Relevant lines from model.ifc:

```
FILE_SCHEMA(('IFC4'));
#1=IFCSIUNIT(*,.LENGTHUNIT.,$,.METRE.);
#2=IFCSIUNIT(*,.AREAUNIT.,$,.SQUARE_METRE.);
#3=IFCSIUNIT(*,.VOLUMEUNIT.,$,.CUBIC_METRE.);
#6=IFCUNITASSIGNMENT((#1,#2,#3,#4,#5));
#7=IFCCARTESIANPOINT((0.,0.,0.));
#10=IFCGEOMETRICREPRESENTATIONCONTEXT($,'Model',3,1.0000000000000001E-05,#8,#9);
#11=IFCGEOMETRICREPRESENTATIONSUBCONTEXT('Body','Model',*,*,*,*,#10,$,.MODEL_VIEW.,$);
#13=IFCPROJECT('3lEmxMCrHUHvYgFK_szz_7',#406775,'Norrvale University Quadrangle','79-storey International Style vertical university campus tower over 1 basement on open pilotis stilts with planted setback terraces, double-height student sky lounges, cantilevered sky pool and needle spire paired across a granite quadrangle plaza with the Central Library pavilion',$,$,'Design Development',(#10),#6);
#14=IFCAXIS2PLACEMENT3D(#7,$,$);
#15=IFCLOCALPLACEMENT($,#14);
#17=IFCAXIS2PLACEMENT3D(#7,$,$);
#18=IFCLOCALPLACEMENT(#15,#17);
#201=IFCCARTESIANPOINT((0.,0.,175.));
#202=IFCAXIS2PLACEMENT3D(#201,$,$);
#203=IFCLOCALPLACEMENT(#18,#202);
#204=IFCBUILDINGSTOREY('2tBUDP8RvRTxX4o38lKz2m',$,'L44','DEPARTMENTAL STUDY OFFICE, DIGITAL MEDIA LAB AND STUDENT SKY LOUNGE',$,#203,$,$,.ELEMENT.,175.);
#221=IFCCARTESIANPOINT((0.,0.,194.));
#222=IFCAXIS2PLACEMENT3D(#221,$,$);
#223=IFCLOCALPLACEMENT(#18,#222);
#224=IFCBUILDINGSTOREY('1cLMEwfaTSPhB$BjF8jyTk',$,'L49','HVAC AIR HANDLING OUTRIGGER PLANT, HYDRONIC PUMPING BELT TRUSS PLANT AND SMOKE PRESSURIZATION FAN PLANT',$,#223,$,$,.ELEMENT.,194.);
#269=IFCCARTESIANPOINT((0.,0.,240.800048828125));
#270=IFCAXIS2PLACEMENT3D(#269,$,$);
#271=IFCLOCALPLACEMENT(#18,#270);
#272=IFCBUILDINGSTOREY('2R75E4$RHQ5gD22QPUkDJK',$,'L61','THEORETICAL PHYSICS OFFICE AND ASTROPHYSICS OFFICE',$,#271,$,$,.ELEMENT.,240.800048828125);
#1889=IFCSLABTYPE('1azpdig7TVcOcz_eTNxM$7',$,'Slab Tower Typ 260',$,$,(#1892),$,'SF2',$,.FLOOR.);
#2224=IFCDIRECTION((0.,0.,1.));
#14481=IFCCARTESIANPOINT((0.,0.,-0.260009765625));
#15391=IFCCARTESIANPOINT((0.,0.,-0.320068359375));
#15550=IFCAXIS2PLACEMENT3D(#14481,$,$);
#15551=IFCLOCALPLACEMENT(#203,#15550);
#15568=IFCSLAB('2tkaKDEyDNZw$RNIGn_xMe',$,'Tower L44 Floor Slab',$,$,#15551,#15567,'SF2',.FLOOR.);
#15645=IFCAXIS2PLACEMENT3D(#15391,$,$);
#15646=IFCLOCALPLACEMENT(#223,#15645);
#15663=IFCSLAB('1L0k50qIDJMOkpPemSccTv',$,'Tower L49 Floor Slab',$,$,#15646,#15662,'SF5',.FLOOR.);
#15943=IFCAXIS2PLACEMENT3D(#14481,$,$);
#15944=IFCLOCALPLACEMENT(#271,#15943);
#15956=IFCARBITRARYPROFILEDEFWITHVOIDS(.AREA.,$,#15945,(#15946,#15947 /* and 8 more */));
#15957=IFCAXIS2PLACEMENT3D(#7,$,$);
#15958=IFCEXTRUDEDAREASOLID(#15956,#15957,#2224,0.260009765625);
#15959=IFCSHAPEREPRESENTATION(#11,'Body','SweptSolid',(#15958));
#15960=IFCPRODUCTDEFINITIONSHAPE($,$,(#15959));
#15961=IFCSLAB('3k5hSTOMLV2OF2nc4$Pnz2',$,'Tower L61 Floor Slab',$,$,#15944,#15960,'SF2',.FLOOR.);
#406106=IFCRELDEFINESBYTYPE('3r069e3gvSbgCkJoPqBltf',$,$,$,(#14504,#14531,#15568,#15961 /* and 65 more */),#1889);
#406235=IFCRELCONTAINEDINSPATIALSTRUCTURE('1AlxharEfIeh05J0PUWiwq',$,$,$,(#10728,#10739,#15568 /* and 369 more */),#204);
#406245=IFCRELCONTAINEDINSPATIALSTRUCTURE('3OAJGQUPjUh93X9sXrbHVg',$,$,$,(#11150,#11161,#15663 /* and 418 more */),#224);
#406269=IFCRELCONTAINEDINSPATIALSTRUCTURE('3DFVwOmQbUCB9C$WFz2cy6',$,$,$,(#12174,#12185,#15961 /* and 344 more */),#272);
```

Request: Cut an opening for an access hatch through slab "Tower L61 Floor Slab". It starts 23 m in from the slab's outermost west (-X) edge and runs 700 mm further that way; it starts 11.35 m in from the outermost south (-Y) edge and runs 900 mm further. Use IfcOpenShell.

```python
import numpy as np
import ifcopenshell
import ifcopenshell.api.feature
import ifcopenshell.api.geometry
import ifcopenshell.api.root
import ifcopenshell.geom
import ifcopenshell.util.placement
import ifcopenshell.util.representation
import ifcopenshell.util.shape
import ifcopenshell.util.unit

model = ifcopenshell.open("model.ifc")
unit_scale = ifcopenshell.util.unit.calculate_unit_scale(model)
settings = ifcopenshell.geom.settings()


def volume(element):
    """Net volume in cubic metres, openings subtracted."""
    shape = ifcopenshell.geom.create_shape(settings, element)
    return ifcopenshell.util.shape.get_volume(shape.geometry)


slab = model.by_guid("3k5hSTOMLV2OF2nc4$Pnz2")
before = volume(slab)

# Extent in the slab's own axes, in metres. The edges named are its -X and -Y sides.
slab_shape = ifcopenshell.geom.create_shape(settings, slab)
vertices = ifcopenshell.util.shape.get_vertices(slab_shape.geometry)
x_min, y_min, bottom = vertices.min(axis=0)
top = vertices[:, 2].max()

opening = ifcopenshell.api.root.create_entity(model, ifc_class="IfcOpeningElement", name="Access hatch opening", predefined_type="OPENING")
context = ifcopenshell.util.representation.get_context(model, "Model", "Body", "MODEL_VIEW")
width, depth = 0.7, 0.9
outline = [(0.0, 0.0), (width, 0.0), (width, depth), (0.0, depth), (0.0, 0.0)]
# Overshoot both faces by 50 mm so the cut is clean.
shape = ifcopenshell.api.geometry.add_slab_representation(
    model, context=context, depth=top - bottom + 0.1, polyline=outline
)
ifcopenshell.api.geometry.assign_representation(model, product=opening, representation=shape)

matrix = ifcopenshell.util.placement.get_local_placement(slab.ObjectPlacement)
matrix[:, 3] = matrix @ np.append(np.array([x_min + 23, y_min + 11.35, bottom - 0.05]) / unit_scale, 1.0)
ifcopenshell.api.geometry.edit_object_placement(model, product=opening, matrix=matrix, is_si=False)
ifcopenshell.api.feature.add_feature(model, feature=opening, element=slab)

after = volume(slab)

print(f"slab volume {before:.3f} -> {after:.3f} m3")

model.write("model-out.ifc")
```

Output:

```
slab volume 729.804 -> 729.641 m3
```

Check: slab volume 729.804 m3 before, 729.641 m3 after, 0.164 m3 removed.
